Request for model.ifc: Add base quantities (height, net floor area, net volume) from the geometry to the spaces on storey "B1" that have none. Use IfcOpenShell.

First a look at what the model holds.

```python
import ifcopenshell
import ifcopenshell.util.element
import ifcopenshell.util.unit

model = ifcopenshell.open("model.ifc")
print(model.schema)
for unit_type in ("LENGTHUNIT", "AREAUNIT", "VOLUMEUNIT"):
    print(unit_type, ifcopenshell.util.unit.calculate_unit_scale(model, unit_type))
storey = next(s for s in model.by_type("IfcBuildingStorey") if s.Name == "B1")
spaces = [e for e in ifcopenshell.util.element.get_decomposition(storey) if e.is_a("IfcSpace")]
for e in sorted(spaces, key=lambda e: e.id()):
    print(e.id(), e.is_a(), e.Name, list(ifcopenshell.util.element.get_psets(e, qtos_only=True)), sep=" | ")
```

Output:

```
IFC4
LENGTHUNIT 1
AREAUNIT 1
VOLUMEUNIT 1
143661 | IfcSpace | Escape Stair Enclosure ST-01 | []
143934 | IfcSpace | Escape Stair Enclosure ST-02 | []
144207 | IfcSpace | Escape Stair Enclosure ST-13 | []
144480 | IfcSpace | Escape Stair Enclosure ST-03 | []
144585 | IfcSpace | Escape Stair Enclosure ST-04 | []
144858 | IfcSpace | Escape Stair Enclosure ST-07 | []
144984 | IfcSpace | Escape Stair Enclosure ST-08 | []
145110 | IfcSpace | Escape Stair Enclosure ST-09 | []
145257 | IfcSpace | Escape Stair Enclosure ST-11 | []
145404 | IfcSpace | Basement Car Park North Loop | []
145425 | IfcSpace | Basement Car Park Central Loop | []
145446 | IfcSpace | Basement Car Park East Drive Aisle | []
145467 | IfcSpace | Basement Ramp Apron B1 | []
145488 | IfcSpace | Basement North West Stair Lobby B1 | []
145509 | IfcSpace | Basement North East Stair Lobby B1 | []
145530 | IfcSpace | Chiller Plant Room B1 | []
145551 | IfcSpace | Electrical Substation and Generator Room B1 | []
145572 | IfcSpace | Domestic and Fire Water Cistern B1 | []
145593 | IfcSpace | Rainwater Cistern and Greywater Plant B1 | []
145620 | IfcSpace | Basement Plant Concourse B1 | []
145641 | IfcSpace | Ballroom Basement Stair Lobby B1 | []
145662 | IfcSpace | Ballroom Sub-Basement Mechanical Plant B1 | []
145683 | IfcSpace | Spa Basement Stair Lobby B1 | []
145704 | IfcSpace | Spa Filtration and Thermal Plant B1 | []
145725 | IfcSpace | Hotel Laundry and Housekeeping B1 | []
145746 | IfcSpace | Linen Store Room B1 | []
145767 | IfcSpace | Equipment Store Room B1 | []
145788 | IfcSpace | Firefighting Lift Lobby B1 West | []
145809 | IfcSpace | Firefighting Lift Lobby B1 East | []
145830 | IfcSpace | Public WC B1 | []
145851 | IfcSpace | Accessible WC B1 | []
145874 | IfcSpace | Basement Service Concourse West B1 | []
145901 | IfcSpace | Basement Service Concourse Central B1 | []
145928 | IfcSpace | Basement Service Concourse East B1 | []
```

```python
import ifcopenshell
import ifcopenshell.api.pset
import ifcopenshell.geom
import ifcopenshell.util.element
import ifcopenshell.util.shape
import ifcopenshell.util.unit

model = ifcopenshell.open("model.ifc")
unit_scale = ifcopenshell.util.unit.calculate_unit_scale(model)
area_scale = ifcopenshell.util.unit.calculate_unit_scale(model, "AREAUNIT")
volume_scale = ifcopenshell.util.unit.calculate_unit_scale(model, "VOLUMEUNIT")
settings = ifcopenshell.geom.settings()

storey = next(s for s in model.by_type("IfcBuildingStorey") if s.Name == "B1")
spaces = [e for e in ifcopenshell.util.element.get_decomposition(storey) if e.is_a("IfcSpace")]

for e in sorted(spaces, key=lambda e: e.id()):
    if ifcopenshell.util.element.get_psets(e, qtos_only=True, should_inherit=False):
        continue
    # Geometry comes back in metres, in the element's own axes.
    shape = ifcopenshell.geom.create_shape(settings, e)
    values = {
        "Height": ifcopenshell.util.shape.get_z(shape.geometry) / unit_scale,
        "NetFloorArea": ifcopenshell.util.shape.get_footprint_area(shape.geometry) / area_scale,
        "NetVolume": ifcopenshell.util.shape.get_volume(shape.geometry) / volume_scale,
    }
    qto = ifcopenshell.api.pset.add_qto(model, product=e, name="Qto_SpaceBaseQuantities")
    ifcopenshell.api.pset.edit_qto(model, qto=qto, properties=values)
    print(e.id(), {k: round(v, 3) for k, v in values.items()})

model.write("model_edited.ifc")
```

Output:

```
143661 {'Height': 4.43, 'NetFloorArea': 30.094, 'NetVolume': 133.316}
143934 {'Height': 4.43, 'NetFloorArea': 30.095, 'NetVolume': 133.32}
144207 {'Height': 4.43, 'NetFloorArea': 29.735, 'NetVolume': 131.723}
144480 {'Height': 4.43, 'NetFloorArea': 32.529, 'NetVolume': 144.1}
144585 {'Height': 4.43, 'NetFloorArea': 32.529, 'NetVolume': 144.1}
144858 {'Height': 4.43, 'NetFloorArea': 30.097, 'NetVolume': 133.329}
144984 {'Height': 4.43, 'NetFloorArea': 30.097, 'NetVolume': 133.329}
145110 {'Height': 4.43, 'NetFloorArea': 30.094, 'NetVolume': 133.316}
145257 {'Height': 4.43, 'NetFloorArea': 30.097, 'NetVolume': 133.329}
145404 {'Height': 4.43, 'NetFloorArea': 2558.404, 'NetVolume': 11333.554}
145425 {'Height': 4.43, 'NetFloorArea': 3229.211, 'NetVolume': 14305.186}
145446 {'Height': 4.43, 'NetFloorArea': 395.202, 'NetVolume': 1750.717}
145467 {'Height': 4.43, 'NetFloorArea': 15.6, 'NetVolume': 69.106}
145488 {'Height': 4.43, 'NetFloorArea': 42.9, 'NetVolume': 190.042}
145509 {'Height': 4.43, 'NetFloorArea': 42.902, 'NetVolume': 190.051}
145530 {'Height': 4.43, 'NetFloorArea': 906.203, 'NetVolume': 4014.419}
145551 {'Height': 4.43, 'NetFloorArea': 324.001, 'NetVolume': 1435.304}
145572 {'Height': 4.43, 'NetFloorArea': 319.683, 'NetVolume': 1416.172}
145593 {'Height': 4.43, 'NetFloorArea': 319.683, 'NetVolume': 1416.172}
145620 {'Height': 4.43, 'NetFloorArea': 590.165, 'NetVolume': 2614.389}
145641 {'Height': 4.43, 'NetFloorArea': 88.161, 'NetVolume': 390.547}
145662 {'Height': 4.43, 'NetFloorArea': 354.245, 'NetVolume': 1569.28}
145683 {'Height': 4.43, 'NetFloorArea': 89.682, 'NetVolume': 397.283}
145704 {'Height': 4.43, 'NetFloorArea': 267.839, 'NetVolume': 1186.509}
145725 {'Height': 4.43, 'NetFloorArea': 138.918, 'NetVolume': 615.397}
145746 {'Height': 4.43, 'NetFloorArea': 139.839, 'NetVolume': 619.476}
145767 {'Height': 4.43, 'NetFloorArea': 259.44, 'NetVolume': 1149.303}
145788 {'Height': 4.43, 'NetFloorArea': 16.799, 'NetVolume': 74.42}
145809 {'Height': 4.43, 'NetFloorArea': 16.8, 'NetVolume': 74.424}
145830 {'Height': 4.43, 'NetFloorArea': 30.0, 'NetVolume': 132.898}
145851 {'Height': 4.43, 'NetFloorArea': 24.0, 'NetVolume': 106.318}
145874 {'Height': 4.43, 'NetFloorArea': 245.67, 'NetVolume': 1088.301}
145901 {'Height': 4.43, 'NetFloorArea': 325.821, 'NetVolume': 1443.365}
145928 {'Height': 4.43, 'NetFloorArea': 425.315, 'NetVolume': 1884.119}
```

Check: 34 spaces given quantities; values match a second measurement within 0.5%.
